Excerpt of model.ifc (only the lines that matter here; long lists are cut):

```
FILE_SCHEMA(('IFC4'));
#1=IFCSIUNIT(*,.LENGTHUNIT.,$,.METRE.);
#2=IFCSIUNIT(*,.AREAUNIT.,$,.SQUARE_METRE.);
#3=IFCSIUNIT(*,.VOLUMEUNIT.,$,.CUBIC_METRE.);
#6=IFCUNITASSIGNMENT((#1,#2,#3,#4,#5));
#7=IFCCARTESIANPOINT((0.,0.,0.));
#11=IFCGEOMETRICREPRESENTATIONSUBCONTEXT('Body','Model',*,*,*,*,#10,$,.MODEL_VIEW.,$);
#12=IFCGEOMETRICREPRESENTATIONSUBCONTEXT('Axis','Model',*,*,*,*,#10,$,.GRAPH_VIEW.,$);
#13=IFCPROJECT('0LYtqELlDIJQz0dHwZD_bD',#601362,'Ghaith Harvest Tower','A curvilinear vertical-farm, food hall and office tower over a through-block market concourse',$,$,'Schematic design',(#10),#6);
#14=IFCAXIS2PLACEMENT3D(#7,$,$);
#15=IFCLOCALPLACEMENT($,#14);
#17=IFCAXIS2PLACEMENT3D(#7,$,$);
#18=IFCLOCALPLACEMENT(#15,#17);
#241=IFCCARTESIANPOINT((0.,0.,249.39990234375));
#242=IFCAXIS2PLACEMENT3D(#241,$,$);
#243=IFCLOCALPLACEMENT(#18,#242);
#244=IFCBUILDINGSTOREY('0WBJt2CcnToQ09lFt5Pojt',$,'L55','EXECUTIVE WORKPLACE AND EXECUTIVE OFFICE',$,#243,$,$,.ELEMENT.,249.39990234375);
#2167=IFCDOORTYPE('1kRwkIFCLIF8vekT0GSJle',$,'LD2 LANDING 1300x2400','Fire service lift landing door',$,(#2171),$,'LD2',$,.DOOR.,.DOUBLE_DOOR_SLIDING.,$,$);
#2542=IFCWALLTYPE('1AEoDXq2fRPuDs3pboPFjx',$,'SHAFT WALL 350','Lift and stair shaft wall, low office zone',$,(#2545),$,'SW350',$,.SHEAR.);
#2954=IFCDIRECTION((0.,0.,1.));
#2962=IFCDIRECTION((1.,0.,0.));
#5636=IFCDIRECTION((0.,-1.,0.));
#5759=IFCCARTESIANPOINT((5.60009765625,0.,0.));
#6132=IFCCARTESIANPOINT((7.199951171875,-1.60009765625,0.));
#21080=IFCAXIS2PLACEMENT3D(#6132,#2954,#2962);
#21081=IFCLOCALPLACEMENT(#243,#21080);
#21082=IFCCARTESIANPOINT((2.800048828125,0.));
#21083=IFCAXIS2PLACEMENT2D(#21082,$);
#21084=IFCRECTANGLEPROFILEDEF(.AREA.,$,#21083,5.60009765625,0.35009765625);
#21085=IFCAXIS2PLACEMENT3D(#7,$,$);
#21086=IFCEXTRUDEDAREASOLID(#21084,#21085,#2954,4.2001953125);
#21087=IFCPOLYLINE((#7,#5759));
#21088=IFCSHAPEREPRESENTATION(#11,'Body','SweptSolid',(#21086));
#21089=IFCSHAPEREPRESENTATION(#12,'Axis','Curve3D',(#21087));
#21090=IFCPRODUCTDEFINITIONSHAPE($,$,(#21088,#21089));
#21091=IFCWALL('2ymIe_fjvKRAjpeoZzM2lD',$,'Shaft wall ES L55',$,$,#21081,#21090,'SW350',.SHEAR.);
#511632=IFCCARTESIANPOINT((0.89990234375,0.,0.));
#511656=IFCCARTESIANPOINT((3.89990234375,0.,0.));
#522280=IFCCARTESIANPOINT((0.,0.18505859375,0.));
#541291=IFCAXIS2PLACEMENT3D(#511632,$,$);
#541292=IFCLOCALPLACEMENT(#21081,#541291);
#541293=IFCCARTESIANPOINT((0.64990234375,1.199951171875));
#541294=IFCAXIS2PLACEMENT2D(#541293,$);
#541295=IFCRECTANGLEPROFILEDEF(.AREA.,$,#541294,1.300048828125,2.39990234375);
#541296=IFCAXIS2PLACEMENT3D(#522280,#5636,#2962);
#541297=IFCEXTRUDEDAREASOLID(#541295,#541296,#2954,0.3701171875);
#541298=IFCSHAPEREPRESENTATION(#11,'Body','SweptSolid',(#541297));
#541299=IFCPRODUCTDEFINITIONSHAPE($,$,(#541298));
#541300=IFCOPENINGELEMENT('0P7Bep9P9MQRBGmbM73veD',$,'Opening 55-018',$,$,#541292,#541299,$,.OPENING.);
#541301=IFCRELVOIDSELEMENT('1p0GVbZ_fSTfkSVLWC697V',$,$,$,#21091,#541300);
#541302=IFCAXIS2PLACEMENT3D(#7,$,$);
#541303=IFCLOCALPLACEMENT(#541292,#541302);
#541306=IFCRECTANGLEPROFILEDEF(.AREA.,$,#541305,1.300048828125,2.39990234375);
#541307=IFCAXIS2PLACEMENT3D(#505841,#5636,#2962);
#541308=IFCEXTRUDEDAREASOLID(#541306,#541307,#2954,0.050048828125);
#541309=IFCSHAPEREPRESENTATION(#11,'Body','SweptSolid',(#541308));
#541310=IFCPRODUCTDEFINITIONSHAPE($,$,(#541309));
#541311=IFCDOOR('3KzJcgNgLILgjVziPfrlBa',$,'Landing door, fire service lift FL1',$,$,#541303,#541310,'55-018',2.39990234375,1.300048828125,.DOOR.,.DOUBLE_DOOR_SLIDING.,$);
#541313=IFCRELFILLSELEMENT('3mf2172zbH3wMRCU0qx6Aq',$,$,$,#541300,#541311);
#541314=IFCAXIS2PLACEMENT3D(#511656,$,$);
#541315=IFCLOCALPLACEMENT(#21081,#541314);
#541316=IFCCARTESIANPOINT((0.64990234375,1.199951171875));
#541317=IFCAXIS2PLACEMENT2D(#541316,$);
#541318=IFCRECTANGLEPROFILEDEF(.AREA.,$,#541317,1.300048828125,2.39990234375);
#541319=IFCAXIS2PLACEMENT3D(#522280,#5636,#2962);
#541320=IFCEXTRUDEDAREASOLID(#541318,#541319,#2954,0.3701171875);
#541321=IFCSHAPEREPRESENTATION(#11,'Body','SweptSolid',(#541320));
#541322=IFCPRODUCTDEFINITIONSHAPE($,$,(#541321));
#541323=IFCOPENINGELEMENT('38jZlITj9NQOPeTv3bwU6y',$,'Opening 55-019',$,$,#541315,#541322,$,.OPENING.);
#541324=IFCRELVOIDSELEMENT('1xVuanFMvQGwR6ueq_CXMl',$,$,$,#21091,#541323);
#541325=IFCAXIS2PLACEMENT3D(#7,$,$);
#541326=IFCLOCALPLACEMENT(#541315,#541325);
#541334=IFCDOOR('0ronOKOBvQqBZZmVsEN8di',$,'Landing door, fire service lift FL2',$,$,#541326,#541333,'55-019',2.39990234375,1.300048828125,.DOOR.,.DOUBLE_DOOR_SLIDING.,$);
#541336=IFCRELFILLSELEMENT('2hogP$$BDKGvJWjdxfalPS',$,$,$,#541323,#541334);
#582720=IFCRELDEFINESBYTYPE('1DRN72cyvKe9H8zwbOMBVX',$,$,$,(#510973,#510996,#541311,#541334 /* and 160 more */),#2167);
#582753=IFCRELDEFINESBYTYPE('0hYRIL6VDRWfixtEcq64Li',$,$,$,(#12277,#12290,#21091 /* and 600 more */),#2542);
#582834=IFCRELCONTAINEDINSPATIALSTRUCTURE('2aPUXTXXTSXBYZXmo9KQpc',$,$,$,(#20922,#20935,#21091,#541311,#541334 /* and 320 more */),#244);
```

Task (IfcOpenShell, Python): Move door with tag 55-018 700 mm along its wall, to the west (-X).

```python
import ifcopenshell
import ifcopenshell.api.geometry
import ifcopenshell.util.placement
import ifcopenshell.util.unit

model = ifcopenshell.open("model.ifc")
unit_scale = ifcopenshell.util.unit.calculate_unit_scale(model)

door = model.by_guid("3KzJcgNgLILgjVziPfrlBa")
opening = door.FillsVoids[0].RelatingOpeningElement
wall = opening.VoidsElements[0].RelatingBuildingElement

wall_matrix = ifcopenshell.util.placement.get_local_placement(wall.ObjectPlacement)
shift = wall_matrix[:3, 0] * -0.7 / unit_scale
before = ifcopenshell.util.placement.get_local_placement(door.ObjectPlacement)[:3, 3].copy()

# The door is placed relative to its opening, so it follows when the opening moves.
matrix = ifcopenshell.util.placement.get_local_placement(opening.ObjectPlacement)
matrix[:3, 3] += shift
ifcopenshell.api.geometry.edit_object_placement(
    model, product=opening, matrix=matrix, is_si=False, should_transform_children=True
)

after = ifcopenshell.util.placement.get_local_placement(door.ObjectPlacement)[:3, 3]
print("door moved by", (after - before).round(3) + 0.0)

model.write("model-out.ifc")
```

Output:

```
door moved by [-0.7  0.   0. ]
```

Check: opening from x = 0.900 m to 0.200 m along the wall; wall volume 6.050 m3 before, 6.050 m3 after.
